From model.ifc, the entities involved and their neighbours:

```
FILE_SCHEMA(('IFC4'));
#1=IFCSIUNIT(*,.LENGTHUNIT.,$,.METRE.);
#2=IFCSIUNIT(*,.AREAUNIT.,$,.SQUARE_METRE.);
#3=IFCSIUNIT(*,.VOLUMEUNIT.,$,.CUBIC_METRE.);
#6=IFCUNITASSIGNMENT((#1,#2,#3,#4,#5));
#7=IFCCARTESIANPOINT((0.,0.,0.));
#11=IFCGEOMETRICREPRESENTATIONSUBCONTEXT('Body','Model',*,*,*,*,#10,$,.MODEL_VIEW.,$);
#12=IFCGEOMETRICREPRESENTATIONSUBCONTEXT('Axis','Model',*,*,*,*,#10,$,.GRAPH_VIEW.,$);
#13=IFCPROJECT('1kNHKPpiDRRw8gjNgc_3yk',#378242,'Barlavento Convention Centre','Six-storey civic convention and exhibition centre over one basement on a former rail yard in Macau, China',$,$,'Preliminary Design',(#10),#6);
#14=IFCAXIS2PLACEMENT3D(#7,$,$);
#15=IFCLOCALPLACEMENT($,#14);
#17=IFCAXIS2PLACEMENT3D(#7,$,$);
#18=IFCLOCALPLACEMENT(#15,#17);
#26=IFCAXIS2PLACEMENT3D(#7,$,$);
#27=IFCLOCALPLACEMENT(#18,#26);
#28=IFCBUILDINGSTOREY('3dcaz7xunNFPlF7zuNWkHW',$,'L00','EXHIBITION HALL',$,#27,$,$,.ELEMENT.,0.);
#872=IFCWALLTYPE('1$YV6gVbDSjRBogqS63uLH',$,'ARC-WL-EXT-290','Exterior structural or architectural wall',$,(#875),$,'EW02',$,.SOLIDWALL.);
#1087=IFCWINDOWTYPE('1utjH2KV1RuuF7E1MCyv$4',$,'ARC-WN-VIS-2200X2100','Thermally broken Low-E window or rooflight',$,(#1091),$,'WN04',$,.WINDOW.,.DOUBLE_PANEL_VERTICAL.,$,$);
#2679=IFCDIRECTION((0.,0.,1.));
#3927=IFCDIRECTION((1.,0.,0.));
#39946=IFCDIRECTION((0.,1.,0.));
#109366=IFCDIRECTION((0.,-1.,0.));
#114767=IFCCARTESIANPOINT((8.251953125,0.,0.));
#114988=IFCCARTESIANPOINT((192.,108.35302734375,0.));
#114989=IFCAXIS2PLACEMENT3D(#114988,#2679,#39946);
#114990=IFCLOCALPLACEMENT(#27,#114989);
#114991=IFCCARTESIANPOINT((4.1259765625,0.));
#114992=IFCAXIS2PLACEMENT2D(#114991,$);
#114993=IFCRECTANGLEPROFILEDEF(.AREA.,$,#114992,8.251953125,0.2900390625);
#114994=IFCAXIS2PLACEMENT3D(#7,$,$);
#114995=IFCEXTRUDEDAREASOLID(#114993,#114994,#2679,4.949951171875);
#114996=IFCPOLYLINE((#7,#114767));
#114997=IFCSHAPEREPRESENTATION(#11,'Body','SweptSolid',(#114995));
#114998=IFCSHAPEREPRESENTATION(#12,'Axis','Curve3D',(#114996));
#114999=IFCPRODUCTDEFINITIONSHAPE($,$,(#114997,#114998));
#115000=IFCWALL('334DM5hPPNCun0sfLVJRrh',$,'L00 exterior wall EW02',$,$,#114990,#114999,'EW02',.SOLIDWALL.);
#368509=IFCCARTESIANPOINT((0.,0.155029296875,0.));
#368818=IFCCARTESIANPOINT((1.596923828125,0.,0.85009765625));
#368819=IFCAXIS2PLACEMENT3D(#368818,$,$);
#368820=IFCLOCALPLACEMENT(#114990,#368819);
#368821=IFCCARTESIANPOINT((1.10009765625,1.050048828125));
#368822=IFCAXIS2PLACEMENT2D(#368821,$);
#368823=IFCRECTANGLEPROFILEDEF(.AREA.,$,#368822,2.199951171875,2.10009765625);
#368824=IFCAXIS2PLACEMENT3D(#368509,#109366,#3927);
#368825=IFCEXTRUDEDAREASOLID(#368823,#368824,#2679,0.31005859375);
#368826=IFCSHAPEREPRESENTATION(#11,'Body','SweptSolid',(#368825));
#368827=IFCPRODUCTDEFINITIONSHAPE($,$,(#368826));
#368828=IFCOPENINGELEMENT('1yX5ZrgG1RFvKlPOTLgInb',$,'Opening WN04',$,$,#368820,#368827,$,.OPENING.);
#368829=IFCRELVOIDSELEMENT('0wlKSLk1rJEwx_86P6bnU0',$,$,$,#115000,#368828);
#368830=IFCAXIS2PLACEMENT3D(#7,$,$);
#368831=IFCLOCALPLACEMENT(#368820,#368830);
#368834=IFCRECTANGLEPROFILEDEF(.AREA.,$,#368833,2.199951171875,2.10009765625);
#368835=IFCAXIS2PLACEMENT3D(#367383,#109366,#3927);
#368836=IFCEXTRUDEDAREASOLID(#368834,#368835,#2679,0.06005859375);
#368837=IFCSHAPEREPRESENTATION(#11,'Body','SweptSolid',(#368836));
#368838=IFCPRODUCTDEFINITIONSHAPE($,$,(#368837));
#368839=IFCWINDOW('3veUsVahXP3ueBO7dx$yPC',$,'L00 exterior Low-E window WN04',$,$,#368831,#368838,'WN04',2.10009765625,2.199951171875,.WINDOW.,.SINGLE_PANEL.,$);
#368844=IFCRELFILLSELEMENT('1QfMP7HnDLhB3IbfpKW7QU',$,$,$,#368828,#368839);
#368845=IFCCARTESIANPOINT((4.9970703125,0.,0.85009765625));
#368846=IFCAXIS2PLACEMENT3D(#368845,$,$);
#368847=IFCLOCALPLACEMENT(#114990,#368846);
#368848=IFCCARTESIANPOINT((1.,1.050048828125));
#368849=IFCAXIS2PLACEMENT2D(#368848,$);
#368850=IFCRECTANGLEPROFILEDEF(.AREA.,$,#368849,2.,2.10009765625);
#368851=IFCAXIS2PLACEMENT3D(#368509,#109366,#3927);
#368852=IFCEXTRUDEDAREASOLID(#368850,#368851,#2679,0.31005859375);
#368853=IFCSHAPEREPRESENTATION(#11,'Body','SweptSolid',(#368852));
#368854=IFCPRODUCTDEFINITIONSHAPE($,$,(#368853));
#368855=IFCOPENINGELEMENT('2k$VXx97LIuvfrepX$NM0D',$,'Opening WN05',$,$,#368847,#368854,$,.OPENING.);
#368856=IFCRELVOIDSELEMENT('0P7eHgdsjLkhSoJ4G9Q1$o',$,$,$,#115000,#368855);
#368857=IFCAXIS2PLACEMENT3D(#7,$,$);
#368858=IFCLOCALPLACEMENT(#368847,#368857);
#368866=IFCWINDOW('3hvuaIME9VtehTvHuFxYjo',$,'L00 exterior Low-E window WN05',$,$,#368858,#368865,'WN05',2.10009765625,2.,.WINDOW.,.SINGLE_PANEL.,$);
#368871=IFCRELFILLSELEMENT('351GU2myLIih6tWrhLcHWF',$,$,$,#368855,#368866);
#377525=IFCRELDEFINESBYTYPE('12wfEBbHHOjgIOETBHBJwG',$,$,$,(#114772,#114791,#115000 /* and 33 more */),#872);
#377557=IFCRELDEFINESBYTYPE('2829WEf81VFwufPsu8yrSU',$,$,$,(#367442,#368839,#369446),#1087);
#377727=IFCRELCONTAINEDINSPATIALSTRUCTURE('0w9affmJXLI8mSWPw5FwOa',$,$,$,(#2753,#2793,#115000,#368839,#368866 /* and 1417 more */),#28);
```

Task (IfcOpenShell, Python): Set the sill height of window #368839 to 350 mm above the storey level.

```python
import numpy as np
import ifcopenshell
import ifcopenshell.api.geometry
import ifcopenshell.geom
import ifcopenshell.util.element
import ifcopenshell.util.placement
import ifcopenshell.util.shape
import ifcopenshell.util.unit

model = ifcopenshell.open("model.ifc")
unit_scale = ifcopenshell.util.unit.calculate_unit_scale(model)

window = model.by_guid("3veUsVahXP3ueBO7dx$yPC")
opening = window.FillsVoids[0].RelatingOpeningElement
storey = ifcopenshell.util.element.get_container(window, ifc_class="IfcBuildingStorey")
level = ifcopenshell.util.placement.get_local_placement(storey.ObjectPlacement)[2, 3]

# The opening's origin need not be at the sill, so measure its lowest point.
shape = ifcopenshell.geom.create_shape(ifcopenshell.geom.settings(), opening)
bottom = ifcopenshell.util.shape.get_shape_bottom_elevation(shape, shape.geometry) / unit_scale
dz = level + 0.35 - bottom

shift = np.array([0.0, 0.0, dz])
# The window is placed relative to its opening, so it follows when the opening moves.
matrix = ifcopenshell.util.placement.get_local_placement(opening.ObjectPlacement)
matrix[:3, 3] += shift
ifcopenshell.api.geometry.edit_object_placement(
    model, product=opening, matrix=matrix, is_si=False, should_transform_children=True
)

print(f"moved by {dz * unit_scale:+.3f} m")

model.write("model_v2.ifc")
```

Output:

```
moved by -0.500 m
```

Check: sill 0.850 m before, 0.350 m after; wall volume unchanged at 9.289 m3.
